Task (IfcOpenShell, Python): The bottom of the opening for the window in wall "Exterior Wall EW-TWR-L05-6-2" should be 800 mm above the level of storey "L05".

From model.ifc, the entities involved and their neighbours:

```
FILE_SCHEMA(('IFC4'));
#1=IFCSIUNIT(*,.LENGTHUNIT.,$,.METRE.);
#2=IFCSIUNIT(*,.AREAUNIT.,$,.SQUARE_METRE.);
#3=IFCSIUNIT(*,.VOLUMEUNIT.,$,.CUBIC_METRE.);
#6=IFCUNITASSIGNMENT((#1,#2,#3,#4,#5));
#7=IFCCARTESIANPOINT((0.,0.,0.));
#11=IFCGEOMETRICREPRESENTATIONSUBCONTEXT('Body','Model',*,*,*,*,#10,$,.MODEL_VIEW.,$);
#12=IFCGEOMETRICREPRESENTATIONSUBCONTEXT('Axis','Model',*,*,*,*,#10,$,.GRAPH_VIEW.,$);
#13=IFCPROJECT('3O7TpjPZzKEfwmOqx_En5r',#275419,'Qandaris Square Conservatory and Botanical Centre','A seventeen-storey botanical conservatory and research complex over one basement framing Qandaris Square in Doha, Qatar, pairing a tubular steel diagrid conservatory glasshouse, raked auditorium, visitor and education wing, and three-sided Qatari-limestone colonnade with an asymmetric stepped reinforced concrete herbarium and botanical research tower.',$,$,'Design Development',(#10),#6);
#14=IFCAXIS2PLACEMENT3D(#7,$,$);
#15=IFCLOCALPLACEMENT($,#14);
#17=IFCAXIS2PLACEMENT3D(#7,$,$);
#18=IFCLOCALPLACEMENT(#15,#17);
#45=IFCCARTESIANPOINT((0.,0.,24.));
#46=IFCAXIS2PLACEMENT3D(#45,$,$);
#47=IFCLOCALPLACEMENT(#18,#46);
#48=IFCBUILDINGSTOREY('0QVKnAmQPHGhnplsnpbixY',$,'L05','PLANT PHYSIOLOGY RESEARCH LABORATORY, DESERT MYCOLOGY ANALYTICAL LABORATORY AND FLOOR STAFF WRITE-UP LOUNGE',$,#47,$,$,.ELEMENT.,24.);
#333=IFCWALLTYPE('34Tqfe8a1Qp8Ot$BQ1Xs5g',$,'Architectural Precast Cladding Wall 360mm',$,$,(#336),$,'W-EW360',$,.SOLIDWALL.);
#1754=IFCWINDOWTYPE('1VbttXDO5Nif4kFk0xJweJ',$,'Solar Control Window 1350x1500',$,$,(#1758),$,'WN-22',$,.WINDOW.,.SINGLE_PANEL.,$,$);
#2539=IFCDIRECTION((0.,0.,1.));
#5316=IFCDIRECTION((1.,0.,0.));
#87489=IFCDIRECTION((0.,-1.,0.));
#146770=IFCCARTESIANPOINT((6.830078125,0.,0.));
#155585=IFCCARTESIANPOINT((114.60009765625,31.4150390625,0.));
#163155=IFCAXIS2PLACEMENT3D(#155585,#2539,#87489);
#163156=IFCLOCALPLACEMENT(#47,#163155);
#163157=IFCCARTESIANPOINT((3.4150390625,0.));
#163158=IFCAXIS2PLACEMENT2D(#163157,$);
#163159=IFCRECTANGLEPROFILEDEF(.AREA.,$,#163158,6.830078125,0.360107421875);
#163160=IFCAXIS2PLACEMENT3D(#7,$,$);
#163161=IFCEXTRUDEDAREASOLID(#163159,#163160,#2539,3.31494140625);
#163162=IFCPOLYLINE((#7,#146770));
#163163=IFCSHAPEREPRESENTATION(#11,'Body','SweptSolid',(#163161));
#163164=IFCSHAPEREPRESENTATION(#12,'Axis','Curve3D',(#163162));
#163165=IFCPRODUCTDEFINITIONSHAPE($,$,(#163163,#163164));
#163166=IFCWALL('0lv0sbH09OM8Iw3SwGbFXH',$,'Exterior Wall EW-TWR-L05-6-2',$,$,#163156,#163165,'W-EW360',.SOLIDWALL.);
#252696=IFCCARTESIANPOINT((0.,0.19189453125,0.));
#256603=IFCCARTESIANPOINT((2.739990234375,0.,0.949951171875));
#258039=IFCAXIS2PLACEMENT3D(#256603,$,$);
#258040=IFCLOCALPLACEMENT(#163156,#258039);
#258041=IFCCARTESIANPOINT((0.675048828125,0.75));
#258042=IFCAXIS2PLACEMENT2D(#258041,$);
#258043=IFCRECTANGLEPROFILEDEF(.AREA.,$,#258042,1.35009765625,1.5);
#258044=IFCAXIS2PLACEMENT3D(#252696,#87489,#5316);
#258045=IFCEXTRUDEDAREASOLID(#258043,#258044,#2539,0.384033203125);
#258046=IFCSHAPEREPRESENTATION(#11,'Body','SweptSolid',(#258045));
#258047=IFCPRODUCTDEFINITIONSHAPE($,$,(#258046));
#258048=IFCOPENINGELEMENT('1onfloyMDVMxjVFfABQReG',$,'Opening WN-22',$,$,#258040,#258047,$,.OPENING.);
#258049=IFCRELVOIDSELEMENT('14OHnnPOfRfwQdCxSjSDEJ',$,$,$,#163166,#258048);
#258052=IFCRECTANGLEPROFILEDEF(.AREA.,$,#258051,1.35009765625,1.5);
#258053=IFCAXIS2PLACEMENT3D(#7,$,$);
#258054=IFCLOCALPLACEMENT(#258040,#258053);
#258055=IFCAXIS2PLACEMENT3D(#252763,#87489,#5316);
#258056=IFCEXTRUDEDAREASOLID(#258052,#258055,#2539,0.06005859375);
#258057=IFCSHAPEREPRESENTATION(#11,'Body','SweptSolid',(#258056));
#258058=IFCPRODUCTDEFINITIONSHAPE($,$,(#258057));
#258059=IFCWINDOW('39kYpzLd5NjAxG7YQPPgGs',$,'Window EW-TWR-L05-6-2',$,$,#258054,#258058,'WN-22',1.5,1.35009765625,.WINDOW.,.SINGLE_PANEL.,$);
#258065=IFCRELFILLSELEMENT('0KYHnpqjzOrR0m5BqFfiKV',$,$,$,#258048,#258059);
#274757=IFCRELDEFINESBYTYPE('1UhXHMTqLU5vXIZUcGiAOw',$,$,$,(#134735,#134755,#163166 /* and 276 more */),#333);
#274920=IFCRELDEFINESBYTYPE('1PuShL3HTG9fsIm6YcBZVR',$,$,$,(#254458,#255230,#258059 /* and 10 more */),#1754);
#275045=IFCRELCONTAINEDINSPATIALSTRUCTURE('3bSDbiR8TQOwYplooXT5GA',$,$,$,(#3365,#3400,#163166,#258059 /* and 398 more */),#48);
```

```python
import numpy as np
import ifcopenshell
import ifcopenshell.api.geometry
import ifcopenshell.geom
import ifcopenshell.util.element
import ifcopenshell.util.placement
import ifcopenshell.util.shape
import ifcopenshell.util.unit

model = ifcopenshell.open("model.ifc")
unit_scale = ifcopenshell.util.unit.calculate_unit_scale(model)

window = model.by_guid("39kYpzLd5NjAxG7YQPPgGs")
opening = window.FillsVoids[0].RelatingOpeningElement
storey = ifcopenshell.util.element.get_container(window, ifc_class="IfcBuildingStorey")
level = ifcopenshell.util.placement.get_local_placement(storey.ObjectPlacement)[2, 3]

# The opening's origin need not be at the sill, so measure its lowest point.
shape = ifcopenshell.geom.create_shape(ifcopenshell.geom.settings(), opening)
bottom = ifcopenshell.util.shape.get_shape_bottom_elevation(shape, shape.geometry) / unit_scale
dz = level + 0.8 - bottom

shift = np.array([0.0, 0.0, dz])
# The window is placed relative to its opening, so it follows when the opening moves.
matrix = ifcopenshell.util.placement.get_local_placement(opening.ObjectPlacement)
matrix[:3, 3] += shift
ifcopenshell.api.geometry.edit_object_placement(
    model, product=opening, matrix=matrix, is_si=False, should_transform_children=True
)

print(f"moved by {dz * unit_scale:+.3f} m")

model.write("model_edited.ifc")
```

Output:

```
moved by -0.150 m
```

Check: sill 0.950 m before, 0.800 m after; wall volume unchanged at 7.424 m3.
